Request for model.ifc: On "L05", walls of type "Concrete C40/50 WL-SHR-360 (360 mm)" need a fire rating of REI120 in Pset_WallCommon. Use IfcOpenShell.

First a look at what the model holds.

```python
import ifcopenshell
import ifcopenshell.util.element

model = ifcopenshell.open("model.ifc")
print(model.schema)
storey = next(s for s in model.by_type("IfcBuildingStorey") if s.Name == "L05")
walls = [e for e in ifcopenshell.util.element.get_decomposition(storey) if e.is_a("IfcWall")]
seen = {}
for e in walls:
    element_type = ifcopenshell.util.element.get_type(e)
    key = (element_type.Name if element_type != e and element_type else None, ifcopenshell.util.element.get_pset(e, "Pset_WallCommon", "FireRating"))
    seen[key] = seen.get(key, 0) + 1
for (name, value), count in sorted(seen.items(), key=str):
    print(count, "x", name, "|", value)
```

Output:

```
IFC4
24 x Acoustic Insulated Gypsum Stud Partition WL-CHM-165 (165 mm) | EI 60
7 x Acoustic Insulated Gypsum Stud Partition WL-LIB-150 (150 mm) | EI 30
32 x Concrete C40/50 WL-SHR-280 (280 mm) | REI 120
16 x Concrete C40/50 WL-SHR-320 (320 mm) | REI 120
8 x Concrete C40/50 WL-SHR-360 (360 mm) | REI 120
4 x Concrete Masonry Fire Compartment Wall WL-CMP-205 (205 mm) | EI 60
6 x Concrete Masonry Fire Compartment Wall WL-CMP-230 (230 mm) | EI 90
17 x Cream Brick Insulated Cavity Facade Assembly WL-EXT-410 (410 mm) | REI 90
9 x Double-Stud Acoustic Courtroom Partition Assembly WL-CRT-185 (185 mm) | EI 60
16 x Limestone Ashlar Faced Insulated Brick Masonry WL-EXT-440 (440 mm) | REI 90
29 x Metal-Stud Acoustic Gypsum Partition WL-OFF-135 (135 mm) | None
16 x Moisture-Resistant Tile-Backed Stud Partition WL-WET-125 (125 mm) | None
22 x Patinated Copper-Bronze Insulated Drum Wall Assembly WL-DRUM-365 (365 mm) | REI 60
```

```python
import ifcopenshell
import ifcopenshell.api.pset
import ifcopenshell.util.element

model = ifcopenshell.open("model.ifc")

storey = next(s for s in model.by_type("IfcBuildingStorey") if s.Name == "L05")
walls = [e for e in ifcopenshell.util.element.get_decomposition(storey) if e.is_a("IfcWall")]

count = 0
for e in walls:
    element_type = ifcopenshell.util.element.get_type(e)
    if element_type in (None, e) or element_type.Name != "Concrete C40/50 WL-SHR-360 (360 mm)":
        continue
    # add_pset returns the element's existing set when there is one.
    pset = ifcopenshell.api.pset.add_pset(model, product=e, name="Pset_WallCommon")
    ifcopenshell.api.pset.edit_pset(model, pset=pset, properties={"FireRating": "REI120"})
    count += 1

print(count, "walls updated")

model.write("model_updated.ifc")
```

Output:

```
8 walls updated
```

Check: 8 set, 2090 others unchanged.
